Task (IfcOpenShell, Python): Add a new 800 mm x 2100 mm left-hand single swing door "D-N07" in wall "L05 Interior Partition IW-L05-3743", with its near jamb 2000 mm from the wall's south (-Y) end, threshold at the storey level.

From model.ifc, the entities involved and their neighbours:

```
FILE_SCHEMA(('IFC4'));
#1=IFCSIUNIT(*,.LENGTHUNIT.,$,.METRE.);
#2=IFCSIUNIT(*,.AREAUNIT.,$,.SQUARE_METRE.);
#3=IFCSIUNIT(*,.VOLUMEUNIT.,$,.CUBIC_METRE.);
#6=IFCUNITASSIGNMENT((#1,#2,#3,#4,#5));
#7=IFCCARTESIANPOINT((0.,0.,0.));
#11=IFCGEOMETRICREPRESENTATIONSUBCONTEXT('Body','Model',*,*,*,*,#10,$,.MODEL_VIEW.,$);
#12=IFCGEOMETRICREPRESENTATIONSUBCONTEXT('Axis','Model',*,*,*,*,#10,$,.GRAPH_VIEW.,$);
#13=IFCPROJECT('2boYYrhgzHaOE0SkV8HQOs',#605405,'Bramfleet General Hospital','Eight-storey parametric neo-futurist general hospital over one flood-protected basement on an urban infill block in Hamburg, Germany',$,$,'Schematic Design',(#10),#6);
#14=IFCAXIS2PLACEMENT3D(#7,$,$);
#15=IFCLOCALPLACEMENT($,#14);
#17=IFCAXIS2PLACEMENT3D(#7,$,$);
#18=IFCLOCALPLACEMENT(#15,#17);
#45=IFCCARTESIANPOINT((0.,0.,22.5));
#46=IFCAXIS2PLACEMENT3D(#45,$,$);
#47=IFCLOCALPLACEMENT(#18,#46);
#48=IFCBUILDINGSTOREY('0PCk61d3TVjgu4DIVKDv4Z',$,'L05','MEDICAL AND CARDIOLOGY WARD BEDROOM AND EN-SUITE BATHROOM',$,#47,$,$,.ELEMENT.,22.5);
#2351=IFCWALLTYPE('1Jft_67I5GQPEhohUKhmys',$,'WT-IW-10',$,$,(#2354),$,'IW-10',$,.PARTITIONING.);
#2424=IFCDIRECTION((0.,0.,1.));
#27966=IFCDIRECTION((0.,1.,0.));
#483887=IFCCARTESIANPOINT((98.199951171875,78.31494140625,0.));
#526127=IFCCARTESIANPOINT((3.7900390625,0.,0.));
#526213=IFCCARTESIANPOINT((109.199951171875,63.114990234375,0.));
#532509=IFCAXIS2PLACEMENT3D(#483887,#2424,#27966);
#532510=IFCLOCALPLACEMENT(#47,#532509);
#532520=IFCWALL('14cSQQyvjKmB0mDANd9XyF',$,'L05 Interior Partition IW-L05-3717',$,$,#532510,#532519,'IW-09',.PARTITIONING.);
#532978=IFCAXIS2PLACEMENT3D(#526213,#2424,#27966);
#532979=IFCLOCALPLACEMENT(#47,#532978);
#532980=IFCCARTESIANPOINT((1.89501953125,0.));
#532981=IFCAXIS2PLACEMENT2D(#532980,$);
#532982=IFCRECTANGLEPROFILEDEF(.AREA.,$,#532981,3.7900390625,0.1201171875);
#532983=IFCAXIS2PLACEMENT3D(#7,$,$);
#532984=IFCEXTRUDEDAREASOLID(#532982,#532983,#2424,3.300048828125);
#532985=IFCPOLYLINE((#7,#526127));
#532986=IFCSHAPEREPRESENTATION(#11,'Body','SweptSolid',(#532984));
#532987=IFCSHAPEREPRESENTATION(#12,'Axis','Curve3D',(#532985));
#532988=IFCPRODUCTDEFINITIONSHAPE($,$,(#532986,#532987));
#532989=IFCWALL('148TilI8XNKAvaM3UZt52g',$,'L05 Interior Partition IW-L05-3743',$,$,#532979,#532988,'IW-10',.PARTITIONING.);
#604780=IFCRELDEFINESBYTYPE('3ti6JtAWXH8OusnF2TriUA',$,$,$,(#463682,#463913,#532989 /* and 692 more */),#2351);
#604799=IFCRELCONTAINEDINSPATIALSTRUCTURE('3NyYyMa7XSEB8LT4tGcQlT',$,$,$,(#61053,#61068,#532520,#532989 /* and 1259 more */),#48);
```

```python
import numpy as np
import ifcopenshell
import ifcopenshell.api.feature
import ifcopenshell.api.geometry
import ifcopenshell.api.root
import ifcopenshell.api.spatial
import ifcopenshell.geom
import ifcopenshell.util.element
import ifcopenshell.util.placement
import ifcopenshell.util.representation
import ifcopenshell.util.shape
import ifcopenshell.util.unit

model = ifcopenshell.open("model.ifc")
unit_scale = ifcopenshell.util.unit.calculate_unit_scale(model)
settings = ifcopenshell.geom.settings()


def volume(element):
    """Net volume in cubic metres, openings subtracted."""
    shape = ifcopenshell.geom.create_shape(settings, element)
    return ifcopenshell.util.shape.get_volume(shape.geometry)


wall = model.by_guid("148TilI8XNKAvaM3UZt52g")
storey = ifcopenshell.util.element.get_container(wall, ifc_class="IfcBuildingStorey")
context = ifcopenshell.util.representation.get_context(model, "Model", "Body", "MODEL_VIEW")
before = volume(wall)

width, height, from_end, sill = 0.8, 2.1, 2, 0.0  # metres

# The wall runs along its own X axis, and the end named is its -X end.
wall_shape = ifcopenshell.geom.create_shape(settings, wall)
x, y, z = ifcopenshell.util.shape.get_vertices(wall_shape.geometry).T
start = x.min() + from_end
face, thickness = float(y.min()), float(y.max() - y.min())
wall_matrix = ifcopenshell.util.placement.get_local_placement(wall.ObjectPlacement)
level = ifcopenshell.util.placement.get_local_placement(storey.ObjectPlacement)[2, 3]


def in_wall(x, y):
    """Placement at x, y metres in the wall's axes, at sill height."""
    matrix = wall_matrix.copy()
    matrix[:, 3] = wall_matrix @ np.array([x / unit_scale, y / unit_scale, 0.0, 1.0])
    matrix[2, 3] = level + sill / unit_scale
    return matrix


# Opening: a box that overshoots both wall faces by 50 mm.
opening = ifcopenshell.api.root.create_entity(model, ifc_class="IfcOpeningElement", predefined_type="OPENING")
box = ifcopenshell.api.geometry.add_wall_representation(
    model, context=context, length=width, height=height, thickness=thickness + 0.1
)
ifcopenshell.api.geometry.assign_representation(model, product=opening, representation=box)
ifcopenshell.api.geometry.edit_object_placement(model, product=opening, matrix=in_wall(start, face - 0.05), is_si=False)
ifcopenshell.api.feature.add_feature(model, feature=opening, element=wall)

door = ifcopenshell.api.root.create_entity(model, ifc_class="IfcDoor", name="D-N07", predefined_type="DOOR")
door.OverallWidth, door.OverallHeight = width / unit_scale, height / unit_scale
door.OperationType = "SINGLE_SWING_LEFT"
body = ifcopenshell.api.geometry.add_door_representation(
    model,
    context=context,
    overall_width=door.OverallWidth,
    overall_height=door.OverallHeight,
    operation_type="SINGLE_SWING_LEFT",
    lining_properties={"LiningDepth": thickness / unit_scale, "ThresholdDepth": thickness / unit_scale},
)
ifcopenshell.api.geometry.assign_representation(model, product=door, representation=body)
ifcopenshell.api.spatial.assign_container(model, products=[door], relating_structure=storey)
ifcopenshell.api.feature.add_filling(model, opening=opening, element=door)

# The lining spans the wall, so the door starts at the wall face.
ifcopenshell.api.geometry.edit_object_placement(model, product=door, matrix=in_wall(start, face), is_si=False)

after = volume(wall)

print(f"wall volume {before:.3f} -> {after:.3f} m3")

model.write("model_updated.ifc")
```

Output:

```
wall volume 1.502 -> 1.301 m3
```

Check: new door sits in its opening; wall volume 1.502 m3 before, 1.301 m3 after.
